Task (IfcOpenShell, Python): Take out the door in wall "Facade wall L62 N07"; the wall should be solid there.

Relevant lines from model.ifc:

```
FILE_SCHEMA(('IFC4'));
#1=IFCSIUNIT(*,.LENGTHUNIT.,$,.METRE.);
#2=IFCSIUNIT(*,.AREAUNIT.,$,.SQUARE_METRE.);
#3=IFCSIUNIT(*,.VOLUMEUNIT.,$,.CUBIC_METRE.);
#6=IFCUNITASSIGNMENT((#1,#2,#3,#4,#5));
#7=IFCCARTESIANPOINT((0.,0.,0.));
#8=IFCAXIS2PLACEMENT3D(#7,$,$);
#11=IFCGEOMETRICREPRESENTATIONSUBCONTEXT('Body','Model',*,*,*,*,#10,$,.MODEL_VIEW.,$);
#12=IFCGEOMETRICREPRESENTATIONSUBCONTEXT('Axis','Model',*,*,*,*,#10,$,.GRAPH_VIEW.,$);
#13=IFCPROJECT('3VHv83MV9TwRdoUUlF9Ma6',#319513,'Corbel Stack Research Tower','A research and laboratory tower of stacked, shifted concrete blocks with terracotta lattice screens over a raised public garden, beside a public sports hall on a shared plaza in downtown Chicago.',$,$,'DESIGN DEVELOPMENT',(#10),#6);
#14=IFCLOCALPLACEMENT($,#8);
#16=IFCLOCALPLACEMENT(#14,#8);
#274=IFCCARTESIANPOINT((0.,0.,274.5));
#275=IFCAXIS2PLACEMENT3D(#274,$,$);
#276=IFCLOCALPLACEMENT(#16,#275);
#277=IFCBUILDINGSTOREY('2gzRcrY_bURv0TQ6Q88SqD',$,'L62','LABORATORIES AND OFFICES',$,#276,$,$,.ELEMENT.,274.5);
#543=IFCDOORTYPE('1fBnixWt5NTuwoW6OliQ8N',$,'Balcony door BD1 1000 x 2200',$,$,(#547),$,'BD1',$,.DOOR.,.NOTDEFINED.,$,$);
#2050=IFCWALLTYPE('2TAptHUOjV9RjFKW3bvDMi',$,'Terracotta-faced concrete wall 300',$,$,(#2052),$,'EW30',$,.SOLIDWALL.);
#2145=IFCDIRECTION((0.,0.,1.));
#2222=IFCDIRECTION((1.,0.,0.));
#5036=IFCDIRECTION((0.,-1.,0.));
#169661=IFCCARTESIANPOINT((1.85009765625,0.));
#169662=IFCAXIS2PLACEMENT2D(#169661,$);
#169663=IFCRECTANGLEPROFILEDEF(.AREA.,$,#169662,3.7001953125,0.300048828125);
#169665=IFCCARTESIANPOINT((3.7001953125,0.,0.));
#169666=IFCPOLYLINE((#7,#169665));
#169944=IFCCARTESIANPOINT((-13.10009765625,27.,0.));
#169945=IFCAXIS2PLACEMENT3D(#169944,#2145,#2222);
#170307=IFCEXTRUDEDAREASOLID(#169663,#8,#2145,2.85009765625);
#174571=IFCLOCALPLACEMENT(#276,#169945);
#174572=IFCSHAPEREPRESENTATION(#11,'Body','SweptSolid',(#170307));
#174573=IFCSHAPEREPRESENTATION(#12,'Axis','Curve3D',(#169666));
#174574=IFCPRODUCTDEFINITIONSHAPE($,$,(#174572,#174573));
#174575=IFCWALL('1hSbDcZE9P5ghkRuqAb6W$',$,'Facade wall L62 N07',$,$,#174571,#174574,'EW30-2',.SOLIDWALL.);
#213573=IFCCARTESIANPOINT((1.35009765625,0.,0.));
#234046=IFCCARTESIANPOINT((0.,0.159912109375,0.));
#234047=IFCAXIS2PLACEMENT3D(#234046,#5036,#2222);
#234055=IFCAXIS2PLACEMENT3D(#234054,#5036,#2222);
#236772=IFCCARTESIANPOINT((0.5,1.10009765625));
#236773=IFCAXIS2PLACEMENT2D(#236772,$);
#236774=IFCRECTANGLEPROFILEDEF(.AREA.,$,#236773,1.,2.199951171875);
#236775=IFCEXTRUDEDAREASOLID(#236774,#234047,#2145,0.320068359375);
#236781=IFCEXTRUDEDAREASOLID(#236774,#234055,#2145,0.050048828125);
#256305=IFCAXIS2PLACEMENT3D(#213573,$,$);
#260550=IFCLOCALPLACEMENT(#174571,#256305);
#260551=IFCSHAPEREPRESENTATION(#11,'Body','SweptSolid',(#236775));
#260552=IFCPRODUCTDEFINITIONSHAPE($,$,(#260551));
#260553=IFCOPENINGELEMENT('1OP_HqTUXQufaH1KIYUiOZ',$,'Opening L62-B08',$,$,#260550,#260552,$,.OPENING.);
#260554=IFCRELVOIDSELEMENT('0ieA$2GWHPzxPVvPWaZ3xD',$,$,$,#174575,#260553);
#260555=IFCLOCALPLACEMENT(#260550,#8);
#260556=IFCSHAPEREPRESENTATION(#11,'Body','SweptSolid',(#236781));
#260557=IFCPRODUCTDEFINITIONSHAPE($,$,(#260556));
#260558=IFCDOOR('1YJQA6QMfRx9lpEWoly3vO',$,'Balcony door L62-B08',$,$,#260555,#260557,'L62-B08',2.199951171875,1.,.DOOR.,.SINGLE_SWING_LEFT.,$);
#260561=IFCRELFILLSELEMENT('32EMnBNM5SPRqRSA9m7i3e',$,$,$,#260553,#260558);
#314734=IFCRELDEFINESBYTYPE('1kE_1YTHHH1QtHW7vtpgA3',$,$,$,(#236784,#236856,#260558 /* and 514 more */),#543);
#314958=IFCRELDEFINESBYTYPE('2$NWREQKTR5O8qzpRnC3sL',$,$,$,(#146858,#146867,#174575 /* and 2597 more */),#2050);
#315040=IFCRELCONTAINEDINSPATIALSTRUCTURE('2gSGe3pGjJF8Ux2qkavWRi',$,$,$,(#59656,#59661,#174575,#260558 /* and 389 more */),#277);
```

```python
import ifcopenshell
import ifcopenshell.api.feature
import ifcopenshell.api.root
import ifcopenshell.geom
import ifcopenshell.util.shape

model = ifcopenshell.open("model.ifc")
settings = ifcopenshell.geom.settings()


def volume(element):
    """Net volume in cubic metres, openings subtracted."""
    shape = ifcopenshell.geom.create_shape(settings, element)
    return ifcopenshell.util.shape.get_volume(shape.geometry)


door = model.by_id(260558)
opening = door.FillsVoids[0].RelatingOpeningElement
wall = opening.VoidsElements[0].RelatingBuildingElement
before = volume(wall)

ifcopenshell.api.root.remove_product(model, product=door)
ifcopenshell.api.feature.remove_feature(model, feature=opening)

after = volume(wall)

print(f"wall volume {before:.3f} -> {after:.3f} m3")

model.write("model_edited.ifc")
```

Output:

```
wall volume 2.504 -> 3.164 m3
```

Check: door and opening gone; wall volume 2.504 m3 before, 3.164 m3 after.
